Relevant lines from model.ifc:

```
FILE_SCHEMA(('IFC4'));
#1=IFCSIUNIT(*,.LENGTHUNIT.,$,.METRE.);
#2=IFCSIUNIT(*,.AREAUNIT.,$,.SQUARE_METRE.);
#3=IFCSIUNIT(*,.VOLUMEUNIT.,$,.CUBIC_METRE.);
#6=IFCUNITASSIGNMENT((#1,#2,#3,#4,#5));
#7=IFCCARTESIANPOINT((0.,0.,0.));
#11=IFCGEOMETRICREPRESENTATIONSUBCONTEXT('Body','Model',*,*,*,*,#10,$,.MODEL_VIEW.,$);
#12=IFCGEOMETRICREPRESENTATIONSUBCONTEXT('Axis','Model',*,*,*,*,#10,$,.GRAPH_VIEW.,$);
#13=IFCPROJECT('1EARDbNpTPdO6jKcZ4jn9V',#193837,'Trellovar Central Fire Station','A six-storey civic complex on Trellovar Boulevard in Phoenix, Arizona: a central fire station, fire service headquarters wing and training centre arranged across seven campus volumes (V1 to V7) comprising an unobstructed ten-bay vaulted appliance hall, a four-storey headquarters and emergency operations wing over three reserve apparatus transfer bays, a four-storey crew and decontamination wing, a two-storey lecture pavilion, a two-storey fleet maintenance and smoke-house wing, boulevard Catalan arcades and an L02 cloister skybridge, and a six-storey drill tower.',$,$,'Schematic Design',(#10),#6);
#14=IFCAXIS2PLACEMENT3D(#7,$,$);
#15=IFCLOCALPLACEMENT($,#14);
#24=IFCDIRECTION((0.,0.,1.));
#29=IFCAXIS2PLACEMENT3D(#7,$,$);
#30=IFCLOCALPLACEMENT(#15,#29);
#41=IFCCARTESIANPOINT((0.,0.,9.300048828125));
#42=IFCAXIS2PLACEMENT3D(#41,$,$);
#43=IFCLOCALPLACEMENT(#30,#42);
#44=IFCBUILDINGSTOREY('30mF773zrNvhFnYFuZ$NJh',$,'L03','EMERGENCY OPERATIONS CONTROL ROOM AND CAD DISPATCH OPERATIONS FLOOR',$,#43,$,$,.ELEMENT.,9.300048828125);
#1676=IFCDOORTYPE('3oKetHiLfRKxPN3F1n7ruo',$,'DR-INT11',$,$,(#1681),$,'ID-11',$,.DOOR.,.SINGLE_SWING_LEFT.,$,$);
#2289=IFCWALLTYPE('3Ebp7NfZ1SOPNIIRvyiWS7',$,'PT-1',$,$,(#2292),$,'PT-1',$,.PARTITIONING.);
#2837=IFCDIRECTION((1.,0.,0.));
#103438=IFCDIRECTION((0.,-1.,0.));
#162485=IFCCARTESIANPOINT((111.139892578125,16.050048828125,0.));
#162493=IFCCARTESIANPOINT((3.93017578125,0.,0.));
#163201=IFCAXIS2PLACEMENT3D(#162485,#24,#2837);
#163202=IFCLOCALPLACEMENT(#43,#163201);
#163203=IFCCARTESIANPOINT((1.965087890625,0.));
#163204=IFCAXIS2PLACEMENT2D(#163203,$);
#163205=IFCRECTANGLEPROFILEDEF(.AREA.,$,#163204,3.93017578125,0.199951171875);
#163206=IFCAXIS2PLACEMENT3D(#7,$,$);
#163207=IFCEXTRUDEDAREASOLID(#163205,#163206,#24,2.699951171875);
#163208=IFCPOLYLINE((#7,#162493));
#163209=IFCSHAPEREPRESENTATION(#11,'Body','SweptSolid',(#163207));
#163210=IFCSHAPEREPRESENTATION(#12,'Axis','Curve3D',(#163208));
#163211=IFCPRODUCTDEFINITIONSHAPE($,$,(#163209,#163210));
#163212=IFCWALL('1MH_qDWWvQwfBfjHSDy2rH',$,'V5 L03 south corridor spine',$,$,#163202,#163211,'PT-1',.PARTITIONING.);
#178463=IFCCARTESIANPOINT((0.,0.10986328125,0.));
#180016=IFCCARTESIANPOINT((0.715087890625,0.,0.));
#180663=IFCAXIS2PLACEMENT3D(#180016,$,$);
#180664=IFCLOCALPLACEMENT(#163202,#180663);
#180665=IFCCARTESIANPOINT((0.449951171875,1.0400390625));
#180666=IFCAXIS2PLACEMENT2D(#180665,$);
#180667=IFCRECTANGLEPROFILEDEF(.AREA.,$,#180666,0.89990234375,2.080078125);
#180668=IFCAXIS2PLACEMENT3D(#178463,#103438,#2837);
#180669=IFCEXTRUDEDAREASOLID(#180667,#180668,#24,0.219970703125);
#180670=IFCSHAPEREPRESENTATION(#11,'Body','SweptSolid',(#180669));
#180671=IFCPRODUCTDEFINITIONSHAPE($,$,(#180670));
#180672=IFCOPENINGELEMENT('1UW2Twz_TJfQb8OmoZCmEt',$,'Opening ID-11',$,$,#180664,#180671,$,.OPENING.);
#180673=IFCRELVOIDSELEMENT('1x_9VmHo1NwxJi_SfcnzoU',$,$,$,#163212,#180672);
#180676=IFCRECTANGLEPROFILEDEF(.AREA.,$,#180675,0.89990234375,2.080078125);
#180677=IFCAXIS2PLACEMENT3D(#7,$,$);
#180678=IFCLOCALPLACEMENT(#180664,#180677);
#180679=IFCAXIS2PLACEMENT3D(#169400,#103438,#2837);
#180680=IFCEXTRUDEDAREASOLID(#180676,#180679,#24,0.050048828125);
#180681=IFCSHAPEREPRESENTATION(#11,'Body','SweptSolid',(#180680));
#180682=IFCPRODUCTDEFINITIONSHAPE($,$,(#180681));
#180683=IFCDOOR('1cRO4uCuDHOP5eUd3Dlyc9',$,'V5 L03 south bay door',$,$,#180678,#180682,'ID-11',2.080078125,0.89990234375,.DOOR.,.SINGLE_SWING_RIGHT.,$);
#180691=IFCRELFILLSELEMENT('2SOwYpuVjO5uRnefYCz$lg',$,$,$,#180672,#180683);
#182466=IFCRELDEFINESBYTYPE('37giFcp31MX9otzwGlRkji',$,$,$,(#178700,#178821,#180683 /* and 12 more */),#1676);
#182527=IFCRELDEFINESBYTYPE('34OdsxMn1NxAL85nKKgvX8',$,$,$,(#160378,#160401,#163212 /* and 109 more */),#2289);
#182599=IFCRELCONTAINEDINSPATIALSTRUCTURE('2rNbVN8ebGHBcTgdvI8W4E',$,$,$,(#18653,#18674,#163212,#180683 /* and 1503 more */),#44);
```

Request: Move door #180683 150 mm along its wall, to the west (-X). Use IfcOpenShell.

```python
import ifcopenshell
import ifcopenshell.api.geometry
import ifcopenshell.util.placement
import ifcopenshell.util.unit

model = ifcopenshell.open("model.ifc")
unit_scale = ifcopenshell.util.unit.calculate_unit_scale(model)

door = model.by_guid("1cRO4uCuDHOP5eUd3Dlyc9")
opening = door.FillsVoids[0].RelatingOpeningElement
wall = opening.VoidsElements[0].RelatingBuildingElement

wall_matrix = ifcopenshell.util.placement.get_local_placement(wall.ObjectPlacement)
shift = wall_matrix[:3, 0] * -0.15 / unit_scale
before = ifcopenshell.util.placement.get_local_placement(door.ObjectPlacement)[:3, 3].copy()

# The door is placed relative to its opening, so it follows when the opening moves.
matrix = ifcopenshell.util.placement.get_local_placement(opening.ObjectPlacement)
matrix[:3, 3] += shift
ifcopenshell.api.geometry.edit_object_placement(
    model, product=opening, matrix=matrix, is_si=False, should_transform_children=True
)

after = ifcopenshell.util.placement.get_local_placement(door.ObjectPlacement)[:3, 3]
print("door moved by", (after - before).round(3) + 0.0)

model.write("model_v2.ifc")
```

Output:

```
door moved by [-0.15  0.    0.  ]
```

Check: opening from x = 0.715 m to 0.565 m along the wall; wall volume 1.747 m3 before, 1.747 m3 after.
